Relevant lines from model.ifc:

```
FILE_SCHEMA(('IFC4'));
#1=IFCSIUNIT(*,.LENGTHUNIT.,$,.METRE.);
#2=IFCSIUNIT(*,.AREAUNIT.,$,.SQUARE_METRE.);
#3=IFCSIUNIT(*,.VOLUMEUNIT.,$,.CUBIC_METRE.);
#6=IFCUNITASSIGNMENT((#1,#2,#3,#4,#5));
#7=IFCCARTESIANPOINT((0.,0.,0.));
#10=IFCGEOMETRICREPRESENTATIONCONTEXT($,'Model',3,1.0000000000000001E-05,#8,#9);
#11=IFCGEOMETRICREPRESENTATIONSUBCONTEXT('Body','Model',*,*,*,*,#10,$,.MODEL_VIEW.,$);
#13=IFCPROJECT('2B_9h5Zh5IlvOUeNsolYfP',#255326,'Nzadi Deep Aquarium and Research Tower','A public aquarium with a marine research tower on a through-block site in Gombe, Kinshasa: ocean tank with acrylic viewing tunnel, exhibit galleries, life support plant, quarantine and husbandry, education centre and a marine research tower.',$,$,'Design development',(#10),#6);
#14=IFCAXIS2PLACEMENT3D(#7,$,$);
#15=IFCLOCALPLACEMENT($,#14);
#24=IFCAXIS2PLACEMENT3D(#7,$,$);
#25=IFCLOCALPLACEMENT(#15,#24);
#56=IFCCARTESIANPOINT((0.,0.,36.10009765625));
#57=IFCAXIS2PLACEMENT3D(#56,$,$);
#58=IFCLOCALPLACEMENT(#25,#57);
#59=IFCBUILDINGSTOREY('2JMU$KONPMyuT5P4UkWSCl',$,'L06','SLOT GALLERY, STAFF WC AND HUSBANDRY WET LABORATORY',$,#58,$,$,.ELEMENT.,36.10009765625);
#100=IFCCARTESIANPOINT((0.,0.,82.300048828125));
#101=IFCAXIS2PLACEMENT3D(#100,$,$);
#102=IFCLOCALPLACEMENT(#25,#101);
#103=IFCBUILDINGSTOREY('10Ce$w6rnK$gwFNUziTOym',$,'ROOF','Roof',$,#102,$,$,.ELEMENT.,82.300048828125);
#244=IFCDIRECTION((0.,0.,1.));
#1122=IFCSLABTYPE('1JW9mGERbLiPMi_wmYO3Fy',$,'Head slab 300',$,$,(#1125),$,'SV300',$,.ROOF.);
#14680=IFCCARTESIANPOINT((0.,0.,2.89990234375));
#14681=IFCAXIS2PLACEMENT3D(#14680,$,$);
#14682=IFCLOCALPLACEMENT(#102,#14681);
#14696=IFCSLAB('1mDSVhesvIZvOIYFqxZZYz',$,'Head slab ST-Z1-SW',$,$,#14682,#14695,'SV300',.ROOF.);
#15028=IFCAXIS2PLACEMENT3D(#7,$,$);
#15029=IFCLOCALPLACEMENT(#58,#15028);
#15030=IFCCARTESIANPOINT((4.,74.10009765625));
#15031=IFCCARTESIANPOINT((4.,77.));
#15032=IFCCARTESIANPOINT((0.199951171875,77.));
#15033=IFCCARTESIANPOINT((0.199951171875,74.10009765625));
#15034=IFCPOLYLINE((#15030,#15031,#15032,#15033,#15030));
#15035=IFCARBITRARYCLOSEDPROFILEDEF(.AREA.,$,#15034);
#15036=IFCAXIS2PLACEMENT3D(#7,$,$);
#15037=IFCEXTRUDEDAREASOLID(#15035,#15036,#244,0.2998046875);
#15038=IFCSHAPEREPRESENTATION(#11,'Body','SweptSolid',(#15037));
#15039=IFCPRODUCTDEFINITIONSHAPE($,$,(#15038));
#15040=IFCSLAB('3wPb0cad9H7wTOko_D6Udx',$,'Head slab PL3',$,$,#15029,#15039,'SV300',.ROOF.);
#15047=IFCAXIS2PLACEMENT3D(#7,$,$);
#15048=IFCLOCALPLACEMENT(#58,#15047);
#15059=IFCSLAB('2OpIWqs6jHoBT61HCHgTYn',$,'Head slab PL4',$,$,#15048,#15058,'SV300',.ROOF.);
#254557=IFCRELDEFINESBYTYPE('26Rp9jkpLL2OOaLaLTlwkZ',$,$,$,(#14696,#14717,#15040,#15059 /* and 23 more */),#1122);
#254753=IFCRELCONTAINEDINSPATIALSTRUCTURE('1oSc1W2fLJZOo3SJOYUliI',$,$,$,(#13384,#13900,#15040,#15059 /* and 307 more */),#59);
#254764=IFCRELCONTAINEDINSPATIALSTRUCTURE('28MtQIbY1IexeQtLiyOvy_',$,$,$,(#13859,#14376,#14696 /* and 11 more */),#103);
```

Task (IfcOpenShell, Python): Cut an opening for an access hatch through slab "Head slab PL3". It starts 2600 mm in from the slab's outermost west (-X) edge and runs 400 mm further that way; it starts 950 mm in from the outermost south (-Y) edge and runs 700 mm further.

```python
import numpy as np
import ifcopenshell
import ifcopenshell.api.feature
import ifcopenshell.api.geometry
import ifcopenshell.api.root
import ifcopenshell.geom
import ifcopenshell.util.placement
import ifcopenshell.util.representation
import ifcopenshell.util.shape
import ifcopenshell.util.unit

model = ifcopenshell.open("model.ifc")
unit_scale = ifcopenshell.util.unit.calculate_unit_scale(model)
settings = ifcopenshell.geom.settings()


def volume(element):
    """Net volume in cubic metres, openings subtracted."""
    shape = ifcopenshell.geom.create_shape(settings, element)
    return ifcopenshell.util.shape.get_volume(shape.geometry)


slab = model.by_guid("3wPb0cad9H7wTOko_D6Udx")
before = volume(slab)

# Extent in the slab's own axes, in metres. The edges named are its -X and -Y sides.
slab_shape = ifcopenshell.geom.create_shape(settings, slab)
vertices = ifcopenshell.util.shape.get_vertices(slab_shape.geometry)
x_min, y_min, bottom = vertices.min(axis=0)
top = vertices[:, 2].max()

opening = ifcopenshell.api.root.create_entity(model, ifc_class="IfcOpeningElement", name="Access hatch opening", predefined_type="OPENING")
context = ifcopenshell.util.representation.get_context(model, "Model", "Body", "MODEL_VIEW")
width, depth = 0.4, 0.7
outline = [(0.0, 0.0), (width, 0.0), (width, depth), (0.0, depth), (0.0, 0.0)]
# Overshoot both faces by 50 mm so the cut is clean.
shape = ifcopenshell.api.geometry.add_slab_representation(
    model, context=context, depth=top - bottom + 0.1, polyline=outline
)
ifcopenshell.api.geometry.assign_representation(model, product=opening, representation=shape)

matrix = ifcopenshell.util.placement.get_local_placement(slab.ObjectPlacement)
matrix[:, 3] = matrix @ np.append(np.array([x_min + 2.6, y_min + 0.95, bottom - 0.05]) / unit_scale, 1.0)
ifcopenshell.api.geometry.edit_object_placement(model, product=opening, matrix=matrix, is_si=False)
ifcopenshell.api.feature.add_feature(model, feature=opening, element=slab)

after = volume(slab)

print(f"slab volume {before:.3f} -> {after:.3f} m3")

model.write("model_v2.ifc")
```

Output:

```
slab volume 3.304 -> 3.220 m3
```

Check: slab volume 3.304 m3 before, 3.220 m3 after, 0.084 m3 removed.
